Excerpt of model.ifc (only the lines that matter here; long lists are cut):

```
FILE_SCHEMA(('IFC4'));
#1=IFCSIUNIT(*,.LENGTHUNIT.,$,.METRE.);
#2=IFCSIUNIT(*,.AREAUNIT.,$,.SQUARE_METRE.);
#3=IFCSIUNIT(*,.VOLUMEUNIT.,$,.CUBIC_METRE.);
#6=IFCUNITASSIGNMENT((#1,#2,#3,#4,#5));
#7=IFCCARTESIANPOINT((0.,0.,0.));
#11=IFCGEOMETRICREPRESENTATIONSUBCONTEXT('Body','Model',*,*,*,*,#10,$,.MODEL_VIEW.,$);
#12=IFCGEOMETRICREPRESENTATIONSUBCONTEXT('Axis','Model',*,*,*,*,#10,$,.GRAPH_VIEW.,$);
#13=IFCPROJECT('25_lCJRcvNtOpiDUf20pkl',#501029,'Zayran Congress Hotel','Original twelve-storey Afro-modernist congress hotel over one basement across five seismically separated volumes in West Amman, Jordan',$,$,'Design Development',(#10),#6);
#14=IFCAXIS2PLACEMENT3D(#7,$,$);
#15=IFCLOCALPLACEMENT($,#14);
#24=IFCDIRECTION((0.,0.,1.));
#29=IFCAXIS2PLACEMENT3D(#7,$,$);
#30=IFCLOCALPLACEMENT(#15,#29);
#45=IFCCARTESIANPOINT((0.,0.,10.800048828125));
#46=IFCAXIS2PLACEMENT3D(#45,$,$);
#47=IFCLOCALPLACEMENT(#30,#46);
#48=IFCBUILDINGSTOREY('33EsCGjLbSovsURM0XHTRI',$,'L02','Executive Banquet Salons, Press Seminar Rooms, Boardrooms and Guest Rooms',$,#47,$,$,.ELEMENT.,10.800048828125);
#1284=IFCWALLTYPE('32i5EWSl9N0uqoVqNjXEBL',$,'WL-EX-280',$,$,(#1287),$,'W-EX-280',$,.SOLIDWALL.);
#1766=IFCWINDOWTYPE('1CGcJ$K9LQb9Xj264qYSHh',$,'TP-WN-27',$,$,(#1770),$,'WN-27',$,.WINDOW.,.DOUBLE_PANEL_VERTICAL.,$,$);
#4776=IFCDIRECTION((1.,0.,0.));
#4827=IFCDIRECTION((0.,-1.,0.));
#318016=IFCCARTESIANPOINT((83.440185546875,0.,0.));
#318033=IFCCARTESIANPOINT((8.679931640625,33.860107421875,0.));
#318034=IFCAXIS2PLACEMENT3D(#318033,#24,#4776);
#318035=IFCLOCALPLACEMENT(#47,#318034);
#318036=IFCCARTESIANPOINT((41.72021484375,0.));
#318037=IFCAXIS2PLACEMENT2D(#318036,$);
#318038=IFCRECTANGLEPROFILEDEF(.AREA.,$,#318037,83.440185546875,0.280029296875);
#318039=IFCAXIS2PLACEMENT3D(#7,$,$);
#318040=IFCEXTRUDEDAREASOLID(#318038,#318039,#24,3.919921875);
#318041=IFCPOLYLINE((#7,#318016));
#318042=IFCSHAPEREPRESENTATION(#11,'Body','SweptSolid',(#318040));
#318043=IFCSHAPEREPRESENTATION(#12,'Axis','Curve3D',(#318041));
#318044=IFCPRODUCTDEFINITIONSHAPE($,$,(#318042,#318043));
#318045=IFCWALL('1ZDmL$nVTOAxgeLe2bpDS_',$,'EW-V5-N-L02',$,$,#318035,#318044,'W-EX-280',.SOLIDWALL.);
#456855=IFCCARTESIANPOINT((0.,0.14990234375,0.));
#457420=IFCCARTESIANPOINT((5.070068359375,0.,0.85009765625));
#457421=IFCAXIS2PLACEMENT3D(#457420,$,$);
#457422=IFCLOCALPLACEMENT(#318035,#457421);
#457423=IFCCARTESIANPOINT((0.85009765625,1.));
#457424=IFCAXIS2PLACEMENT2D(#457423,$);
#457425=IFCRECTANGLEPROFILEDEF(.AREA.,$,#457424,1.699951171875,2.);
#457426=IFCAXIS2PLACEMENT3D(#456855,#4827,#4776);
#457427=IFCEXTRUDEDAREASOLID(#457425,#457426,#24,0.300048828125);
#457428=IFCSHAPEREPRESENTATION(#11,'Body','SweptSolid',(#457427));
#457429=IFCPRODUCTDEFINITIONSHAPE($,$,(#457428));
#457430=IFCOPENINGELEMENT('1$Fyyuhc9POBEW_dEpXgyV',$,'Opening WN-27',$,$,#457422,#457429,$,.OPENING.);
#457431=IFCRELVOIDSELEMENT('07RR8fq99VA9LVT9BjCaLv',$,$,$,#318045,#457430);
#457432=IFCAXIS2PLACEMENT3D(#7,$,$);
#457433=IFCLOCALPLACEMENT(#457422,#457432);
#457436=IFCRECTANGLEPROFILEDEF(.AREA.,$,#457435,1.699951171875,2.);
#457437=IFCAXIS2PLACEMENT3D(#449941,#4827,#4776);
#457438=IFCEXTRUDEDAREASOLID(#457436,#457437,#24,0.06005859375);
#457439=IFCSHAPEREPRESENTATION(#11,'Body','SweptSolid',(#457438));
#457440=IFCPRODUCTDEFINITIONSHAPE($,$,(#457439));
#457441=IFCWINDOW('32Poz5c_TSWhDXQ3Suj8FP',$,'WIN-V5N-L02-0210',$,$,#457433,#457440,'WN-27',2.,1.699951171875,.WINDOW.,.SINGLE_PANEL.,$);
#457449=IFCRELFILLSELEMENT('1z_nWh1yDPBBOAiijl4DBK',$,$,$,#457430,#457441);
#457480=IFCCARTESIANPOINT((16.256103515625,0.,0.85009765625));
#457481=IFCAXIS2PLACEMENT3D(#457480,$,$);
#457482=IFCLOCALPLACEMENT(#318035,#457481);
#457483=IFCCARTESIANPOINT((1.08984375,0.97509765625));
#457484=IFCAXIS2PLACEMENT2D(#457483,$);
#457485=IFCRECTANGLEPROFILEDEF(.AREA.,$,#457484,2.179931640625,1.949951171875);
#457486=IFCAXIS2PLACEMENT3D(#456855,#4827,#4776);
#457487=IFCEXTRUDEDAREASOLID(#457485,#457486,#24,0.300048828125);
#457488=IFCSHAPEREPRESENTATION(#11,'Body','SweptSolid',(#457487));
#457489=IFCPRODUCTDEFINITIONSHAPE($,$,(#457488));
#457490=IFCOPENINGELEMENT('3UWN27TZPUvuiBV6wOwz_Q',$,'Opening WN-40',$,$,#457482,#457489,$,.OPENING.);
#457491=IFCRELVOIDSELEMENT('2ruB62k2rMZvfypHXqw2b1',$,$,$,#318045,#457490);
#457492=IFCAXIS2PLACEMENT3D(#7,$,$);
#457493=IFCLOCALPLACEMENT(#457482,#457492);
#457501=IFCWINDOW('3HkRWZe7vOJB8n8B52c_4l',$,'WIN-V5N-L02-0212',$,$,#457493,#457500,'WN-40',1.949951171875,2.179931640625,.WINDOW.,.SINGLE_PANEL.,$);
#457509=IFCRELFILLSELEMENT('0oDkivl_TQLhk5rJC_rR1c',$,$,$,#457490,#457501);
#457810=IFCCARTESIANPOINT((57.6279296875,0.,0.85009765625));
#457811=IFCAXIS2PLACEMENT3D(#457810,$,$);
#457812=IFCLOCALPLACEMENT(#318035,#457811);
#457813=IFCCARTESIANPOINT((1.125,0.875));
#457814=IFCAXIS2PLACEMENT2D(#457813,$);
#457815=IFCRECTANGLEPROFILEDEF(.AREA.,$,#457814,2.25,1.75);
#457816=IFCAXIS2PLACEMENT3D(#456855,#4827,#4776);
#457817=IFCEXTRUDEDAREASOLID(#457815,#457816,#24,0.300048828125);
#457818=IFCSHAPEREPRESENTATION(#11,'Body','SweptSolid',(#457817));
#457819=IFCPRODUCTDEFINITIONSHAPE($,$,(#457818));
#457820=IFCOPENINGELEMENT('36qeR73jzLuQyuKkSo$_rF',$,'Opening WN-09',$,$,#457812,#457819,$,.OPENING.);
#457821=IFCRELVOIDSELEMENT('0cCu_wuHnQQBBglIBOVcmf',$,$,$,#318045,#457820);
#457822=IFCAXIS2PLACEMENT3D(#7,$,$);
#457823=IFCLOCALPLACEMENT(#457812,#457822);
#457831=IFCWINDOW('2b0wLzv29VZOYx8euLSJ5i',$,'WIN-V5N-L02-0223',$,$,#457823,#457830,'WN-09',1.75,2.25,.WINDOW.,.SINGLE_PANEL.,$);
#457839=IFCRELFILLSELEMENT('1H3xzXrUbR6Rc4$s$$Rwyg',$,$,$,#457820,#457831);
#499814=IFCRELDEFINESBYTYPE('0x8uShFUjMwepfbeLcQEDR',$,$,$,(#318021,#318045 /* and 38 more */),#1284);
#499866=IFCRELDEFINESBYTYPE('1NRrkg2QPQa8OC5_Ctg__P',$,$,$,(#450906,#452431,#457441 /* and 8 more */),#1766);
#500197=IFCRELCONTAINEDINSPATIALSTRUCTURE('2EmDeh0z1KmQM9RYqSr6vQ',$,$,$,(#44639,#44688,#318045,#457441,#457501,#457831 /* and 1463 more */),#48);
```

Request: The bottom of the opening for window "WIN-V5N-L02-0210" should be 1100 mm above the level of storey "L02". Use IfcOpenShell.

```python
import numpy as np
import ifcopenshell
import ifcopenshell.api.geometry
import ifcopenshell.geom
import ifcopenshell.util.element
import ifcopenshell.util.placement
import ifcopenshell.util.shape
import ifcopenshell.util.unit

model = ifcopenshell.open("model.ifc")
unit_scale = ifcopenshell.util.unit.calculate_unit_scale(model)

window = model.by_id(457441)
opening = window.FillsVoids[0].RelatingOpeningElement
storey = ifcopenshell.util.element.get_container(window, ifc_class="IfcBuildingStorey")
level = ifcopenshell.util.placement.get_local_placement(storey.ObjectPlacement)[2, 3]

# The opening's origin need not be at the sill, so measure its lowest point.
shape = ifcopenshell.geom.create_shape(ifcopenshell.geom.settings(), opening)
bottom = ifcopenshell.util.shape.get_shape_bottom_elevation(shape, shape.geometry) / unit_scale
dz = level + 1.1 - bottom

shift = np.array([0.0, 0.0, dz])
# The window is placed relative to its opening, so it follows when the opening moves.
matrix = ifcopenshell.util.placement.get_local_placement(opening.ObjectPlacement)
matrix[:3, 3] += shift
ifcopenshell.api.geometry.edit_object_placement(
    model, product=opening, matrix=matrix, is_si=False, should_transform_children=True
)

print(f"moved by {dz * unit_scale:+.3f} m")

model.write("model_v2.ifc")
```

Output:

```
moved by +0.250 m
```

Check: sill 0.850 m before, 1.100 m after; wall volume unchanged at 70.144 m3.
